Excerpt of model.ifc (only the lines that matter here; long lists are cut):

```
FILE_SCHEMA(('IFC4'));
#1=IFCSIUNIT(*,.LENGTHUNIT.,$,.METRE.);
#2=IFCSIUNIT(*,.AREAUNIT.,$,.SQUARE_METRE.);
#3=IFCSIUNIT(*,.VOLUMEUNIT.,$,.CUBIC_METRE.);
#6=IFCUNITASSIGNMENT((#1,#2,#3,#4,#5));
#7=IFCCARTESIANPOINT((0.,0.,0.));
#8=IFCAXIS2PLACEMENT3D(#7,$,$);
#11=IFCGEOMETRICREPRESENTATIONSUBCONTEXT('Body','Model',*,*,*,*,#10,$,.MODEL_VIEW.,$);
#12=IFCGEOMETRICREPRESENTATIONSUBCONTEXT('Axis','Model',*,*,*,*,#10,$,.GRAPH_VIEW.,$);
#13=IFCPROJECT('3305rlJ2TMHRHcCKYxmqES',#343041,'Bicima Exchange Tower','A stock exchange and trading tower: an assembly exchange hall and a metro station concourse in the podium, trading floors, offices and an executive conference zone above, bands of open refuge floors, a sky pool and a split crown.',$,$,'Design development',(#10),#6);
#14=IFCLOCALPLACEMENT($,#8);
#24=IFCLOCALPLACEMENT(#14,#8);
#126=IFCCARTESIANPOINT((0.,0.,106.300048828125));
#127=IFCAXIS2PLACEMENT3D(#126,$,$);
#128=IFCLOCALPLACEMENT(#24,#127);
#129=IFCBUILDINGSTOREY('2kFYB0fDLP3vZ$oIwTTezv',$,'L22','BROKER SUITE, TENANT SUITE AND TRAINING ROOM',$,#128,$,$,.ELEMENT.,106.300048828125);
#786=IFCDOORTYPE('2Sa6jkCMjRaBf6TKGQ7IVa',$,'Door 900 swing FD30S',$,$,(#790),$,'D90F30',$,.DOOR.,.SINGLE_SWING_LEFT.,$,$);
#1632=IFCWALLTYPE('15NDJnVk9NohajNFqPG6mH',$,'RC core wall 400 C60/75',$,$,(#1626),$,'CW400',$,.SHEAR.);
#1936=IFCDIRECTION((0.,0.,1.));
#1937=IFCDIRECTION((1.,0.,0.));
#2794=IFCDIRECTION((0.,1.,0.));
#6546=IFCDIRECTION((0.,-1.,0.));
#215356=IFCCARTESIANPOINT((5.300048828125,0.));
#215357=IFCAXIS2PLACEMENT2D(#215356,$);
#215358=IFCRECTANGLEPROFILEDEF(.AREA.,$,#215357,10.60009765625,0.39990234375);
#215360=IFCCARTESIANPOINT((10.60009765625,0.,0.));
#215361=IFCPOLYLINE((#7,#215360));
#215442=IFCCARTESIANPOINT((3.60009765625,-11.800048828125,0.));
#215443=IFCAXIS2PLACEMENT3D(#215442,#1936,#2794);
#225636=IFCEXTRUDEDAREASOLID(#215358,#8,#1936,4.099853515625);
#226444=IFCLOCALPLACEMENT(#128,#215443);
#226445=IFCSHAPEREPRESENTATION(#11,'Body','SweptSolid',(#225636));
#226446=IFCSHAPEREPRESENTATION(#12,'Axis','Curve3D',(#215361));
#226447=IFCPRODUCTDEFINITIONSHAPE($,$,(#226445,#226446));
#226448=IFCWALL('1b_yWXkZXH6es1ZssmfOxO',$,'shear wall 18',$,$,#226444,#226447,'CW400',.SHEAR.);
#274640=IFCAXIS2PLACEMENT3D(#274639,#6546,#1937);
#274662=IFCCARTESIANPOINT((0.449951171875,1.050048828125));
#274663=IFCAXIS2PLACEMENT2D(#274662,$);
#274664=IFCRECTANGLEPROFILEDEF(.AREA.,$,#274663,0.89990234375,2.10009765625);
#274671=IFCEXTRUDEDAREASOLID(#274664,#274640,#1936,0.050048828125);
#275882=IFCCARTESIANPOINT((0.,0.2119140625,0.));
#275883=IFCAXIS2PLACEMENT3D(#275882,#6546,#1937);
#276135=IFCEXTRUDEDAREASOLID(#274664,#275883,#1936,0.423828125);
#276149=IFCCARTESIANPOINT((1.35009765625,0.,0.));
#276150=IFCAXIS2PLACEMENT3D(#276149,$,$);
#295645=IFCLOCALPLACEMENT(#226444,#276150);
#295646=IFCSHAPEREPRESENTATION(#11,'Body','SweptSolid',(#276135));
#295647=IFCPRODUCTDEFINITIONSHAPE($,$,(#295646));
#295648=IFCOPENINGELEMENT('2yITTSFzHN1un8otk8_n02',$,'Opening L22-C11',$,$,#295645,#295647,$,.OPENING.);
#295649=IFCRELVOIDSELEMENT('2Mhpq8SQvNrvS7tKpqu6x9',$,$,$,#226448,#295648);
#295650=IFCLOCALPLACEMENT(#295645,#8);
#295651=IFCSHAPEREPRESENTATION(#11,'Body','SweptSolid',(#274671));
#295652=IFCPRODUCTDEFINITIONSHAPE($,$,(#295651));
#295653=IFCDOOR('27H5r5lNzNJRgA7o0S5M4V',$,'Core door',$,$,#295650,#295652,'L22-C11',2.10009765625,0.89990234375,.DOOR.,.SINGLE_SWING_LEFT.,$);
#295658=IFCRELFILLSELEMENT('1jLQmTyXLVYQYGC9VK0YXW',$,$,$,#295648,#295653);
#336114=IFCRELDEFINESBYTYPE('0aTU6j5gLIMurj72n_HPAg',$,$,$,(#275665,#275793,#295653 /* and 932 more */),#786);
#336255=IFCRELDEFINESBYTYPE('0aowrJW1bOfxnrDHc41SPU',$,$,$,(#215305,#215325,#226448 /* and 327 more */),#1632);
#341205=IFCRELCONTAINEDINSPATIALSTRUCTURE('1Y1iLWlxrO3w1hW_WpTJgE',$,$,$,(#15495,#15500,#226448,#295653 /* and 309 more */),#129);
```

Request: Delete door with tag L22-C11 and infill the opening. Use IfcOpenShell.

```python
import ifcopenshell
import ifcopenshell.api.feature
import ifcopenshell.api.root
import ifcopenshell.geom
import ifcopenshell.util.shape

model = ifcopenshell.open("model.ifc")
settings = ifcopenshell.geom.settings()


def volume(element):
    """Net volume in cubic metres, openings subtracted."""
    shape = ifcopenshell.geom.create_shape(settings, element)
    return ifcopenshell.util.shape.get_volume(shape.geometry)


door = model.by_guid("27H5r5lNzNJRgA7o0S5M4V")
opening = door.FillsVoids[0].RelatingOpeningElement
wall = opening.VoidsElements[0].RelatingBuildingElement
before = volume(wall)

ifcopenshell.api.root.remove_product(model, product=door)
ifcopenshell.api.feature.remove_feature(model, feature=opening)

after = volume(wall)

print(f"wall volume {before:.3f} -> {after:.3f} m3")

model.write("model_edited.ifc")
```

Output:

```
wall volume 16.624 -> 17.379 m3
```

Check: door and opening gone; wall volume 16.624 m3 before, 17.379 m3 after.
